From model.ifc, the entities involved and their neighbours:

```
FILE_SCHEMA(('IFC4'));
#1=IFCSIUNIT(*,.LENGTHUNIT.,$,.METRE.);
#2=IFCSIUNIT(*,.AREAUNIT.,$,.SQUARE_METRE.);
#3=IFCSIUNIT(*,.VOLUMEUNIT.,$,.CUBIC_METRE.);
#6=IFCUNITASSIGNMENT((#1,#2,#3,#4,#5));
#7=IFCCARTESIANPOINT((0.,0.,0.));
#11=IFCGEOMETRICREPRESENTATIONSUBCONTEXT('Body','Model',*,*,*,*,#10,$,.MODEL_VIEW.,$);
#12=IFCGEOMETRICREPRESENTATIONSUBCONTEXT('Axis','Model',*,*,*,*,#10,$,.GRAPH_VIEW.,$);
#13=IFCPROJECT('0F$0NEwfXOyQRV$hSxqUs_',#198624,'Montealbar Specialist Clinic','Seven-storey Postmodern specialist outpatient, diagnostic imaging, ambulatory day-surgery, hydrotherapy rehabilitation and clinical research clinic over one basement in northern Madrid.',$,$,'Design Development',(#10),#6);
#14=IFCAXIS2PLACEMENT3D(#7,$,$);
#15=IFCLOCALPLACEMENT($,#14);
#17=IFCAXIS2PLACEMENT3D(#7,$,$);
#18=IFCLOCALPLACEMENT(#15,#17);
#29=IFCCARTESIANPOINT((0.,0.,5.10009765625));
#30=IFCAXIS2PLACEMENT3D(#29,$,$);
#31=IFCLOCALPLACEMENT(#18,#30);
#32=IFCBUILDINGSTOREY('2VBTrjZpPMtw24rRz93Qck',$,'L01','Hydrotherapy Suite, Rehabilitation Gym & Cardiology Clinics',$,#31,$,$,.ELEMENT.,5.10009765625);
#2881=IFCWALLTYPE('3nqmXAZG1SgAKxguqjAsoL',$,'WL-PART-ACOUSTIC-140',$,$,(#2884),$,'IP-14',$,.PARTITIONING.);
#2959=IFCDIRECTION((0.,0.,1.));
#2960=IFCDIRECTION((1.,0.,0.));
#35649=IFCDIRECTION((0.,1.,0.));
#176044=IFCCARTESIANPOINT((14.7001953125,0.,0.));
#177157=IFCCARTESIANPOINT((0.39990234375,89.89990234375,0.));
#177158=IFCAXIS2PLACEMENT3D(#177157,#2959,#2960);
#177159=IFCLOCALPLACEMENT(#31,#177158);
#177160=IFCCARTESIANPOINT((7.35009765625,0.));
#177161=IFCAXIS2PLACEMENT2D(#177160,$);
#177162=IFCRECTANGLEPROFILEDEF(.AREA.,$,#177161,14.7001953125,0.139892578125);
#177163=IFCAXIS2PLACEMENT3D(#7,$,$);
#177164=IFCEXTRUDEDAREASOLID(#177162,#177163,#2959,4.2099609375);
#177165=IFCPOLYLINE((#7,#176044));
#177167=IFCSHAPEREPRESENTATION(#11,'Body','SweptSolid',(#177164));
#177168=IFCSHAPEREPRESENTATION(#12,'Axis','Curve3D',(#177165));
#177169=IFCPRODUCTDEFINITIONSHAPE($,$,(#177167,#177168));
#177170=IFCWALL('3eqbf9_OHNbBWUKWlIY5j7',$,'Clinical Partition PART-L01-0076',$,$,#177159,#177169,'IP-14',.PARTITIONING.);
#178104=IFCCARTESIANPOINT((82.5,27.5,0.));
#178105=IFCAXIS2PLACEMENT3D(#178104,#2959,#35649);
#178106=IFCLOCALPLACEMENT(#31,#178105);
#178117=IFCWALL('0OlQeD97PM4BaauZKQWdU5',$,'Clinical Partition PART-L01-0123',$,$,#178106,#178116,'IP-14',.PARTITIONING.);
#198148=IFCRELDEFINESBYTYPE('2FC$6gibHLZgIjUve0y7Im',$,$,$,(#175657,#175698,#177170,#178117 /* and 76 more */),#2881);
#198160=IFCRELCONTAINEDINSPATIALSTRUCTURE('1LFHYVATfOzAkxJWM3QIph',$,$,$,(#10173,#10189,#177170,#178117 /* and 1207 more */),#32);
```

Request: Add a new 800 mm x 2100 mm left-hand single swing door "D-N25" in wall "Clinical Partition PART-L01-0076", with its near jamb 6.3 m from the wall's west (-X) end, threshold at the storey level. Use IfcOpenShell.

```python
import numpy as np
import ifcopenshell
import ifcopenshell.api.feature
import ifcopenshell.api.geometry
import ifcopenshell.api.root
import ifcopenshell.api.spatial
import ifcopenshell.geom
import ifcopenshell.util.element
import ifcopenshell.util.placement
import ifcopenshell.util.representation
import ifcopenshell.util.shape
import ifcopenshell.util.unit

model = ifcopenshell.open("model.ifc")
unit_scale = ifcopenshell.util.unit.calculate_unit_scale(model)
settings = ifcopenshell.geom.settings()


def volume(element):
    """Net volume in cubic metres, openings subtracted."""
    shape = ifcopenshell.geom.create_shape(settings, element)
    return ifcopenshell.util.shape.get_volume(shape.geometry)


wall = model.by_guid("3eqbf9_OHNbBWUKWlIY5j7")
storey = ifcopenshell.util.element.get_container(wall, ifc_class="IfcBuildingStorey")
context = ifcopenshell.util.representation.get_context(model, "Model", "Body", "MODEL_VIEW")
before = volume(wall)

width, height, from_end, sill = 0.8, 2.1, 6.3, 0.0  # metres

# The wall runs along its own X axis, and the end named is its -X end.
wall_shape = ifcopenshell.geom.create_shape(settings, wall)
x, y, z = ifcopenshell.util.shape.get_vertices(wall_shape.geometry).T
start = x.min() + from_end
face, thickness = float(y.min()), float(y.max() - y.min())
wall_matrix = ifcopenshell.util.placement.get_local_placement(wall.ObjectPlacement)
level = ifcopenshell.util.placement.get_local_placement(storey.ObjectPlacement)[2, 3]


def in_wall(x, y):
    """Placement at x, y metres in the wall's axes, at sill height."""
    matrix = wall_matrix.copy()
    matrix[:, 3] = wall_matrix @ np.array([x / unit_scale, y / unit_scale, 0.0, 1.0])
    matrix[2, 3] = level + sill / unit_scale
    return matrix


# Opening: a box that overshoots both wall faces by 50 mm.
opening = ifcopenshell.api.root.create_entity(model, ifc_class="IfcOpeningElement", predefined_type="OPENING")
box = ifcopenshell.api.geometry.add_wall_representation(
    model, context=context, length=width, height=height, thickness=thickness + 0.1
)
ifcopenshell.api.geometry.assign_representation(model, product=opening, representation=box)
ifcopenshell.api.geometry.edit_object_placement(model, product=opening, matrix=in_wall(start, face - 0.05), is_si=False)
ifcopenshell.api.feature.add_feature(model, feature=opening, element=wall)

door = ifcopenshell.api.root.create_entity(model, ifc_class="IfcDoor", name="D-N25", predefined_type="DOOR")
door.OverallWidth, door.OverallHeight = width / unit_scale, height / unit_scale
door.OperationType = "SINGLE_SWING_LEFT"
body = ifcopenshell.api.geometry.add_door_representation(
    model,
    context=context,
    overall_width=door.OverallWidth,
    overall_height=door.OverallHeight,
    operation_type="SINGLE_SWING_LEFT",
    lining_properties={"LiningDepth": thickness / unit_scale, "ThresholdDepth": thickness / unit_scale},
)
ifcopenshell.api.geometry.assign_representation(model, product=door, representation=body)
ifcopenshell.api.spatial.assign_container(model, products=[door], relating_structure=storey)
ifcopenshell.api.feature.add_filling(model, opening=opening, element=door)

# The lining spans the wall, so the door starts at the wall face.
ifcopenshell.api.geometry.edit_object_placement(model, product=door, matrix=in_wall(start, face), is_si=False)

after = volume(wall)

print(f"wall volume {before:.3f} -> {after:.3f} m3")

model.write("model_edited.ifc")
```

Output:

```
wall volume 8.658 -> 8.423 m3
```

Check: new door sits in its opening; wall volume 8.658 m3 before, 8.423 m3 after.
